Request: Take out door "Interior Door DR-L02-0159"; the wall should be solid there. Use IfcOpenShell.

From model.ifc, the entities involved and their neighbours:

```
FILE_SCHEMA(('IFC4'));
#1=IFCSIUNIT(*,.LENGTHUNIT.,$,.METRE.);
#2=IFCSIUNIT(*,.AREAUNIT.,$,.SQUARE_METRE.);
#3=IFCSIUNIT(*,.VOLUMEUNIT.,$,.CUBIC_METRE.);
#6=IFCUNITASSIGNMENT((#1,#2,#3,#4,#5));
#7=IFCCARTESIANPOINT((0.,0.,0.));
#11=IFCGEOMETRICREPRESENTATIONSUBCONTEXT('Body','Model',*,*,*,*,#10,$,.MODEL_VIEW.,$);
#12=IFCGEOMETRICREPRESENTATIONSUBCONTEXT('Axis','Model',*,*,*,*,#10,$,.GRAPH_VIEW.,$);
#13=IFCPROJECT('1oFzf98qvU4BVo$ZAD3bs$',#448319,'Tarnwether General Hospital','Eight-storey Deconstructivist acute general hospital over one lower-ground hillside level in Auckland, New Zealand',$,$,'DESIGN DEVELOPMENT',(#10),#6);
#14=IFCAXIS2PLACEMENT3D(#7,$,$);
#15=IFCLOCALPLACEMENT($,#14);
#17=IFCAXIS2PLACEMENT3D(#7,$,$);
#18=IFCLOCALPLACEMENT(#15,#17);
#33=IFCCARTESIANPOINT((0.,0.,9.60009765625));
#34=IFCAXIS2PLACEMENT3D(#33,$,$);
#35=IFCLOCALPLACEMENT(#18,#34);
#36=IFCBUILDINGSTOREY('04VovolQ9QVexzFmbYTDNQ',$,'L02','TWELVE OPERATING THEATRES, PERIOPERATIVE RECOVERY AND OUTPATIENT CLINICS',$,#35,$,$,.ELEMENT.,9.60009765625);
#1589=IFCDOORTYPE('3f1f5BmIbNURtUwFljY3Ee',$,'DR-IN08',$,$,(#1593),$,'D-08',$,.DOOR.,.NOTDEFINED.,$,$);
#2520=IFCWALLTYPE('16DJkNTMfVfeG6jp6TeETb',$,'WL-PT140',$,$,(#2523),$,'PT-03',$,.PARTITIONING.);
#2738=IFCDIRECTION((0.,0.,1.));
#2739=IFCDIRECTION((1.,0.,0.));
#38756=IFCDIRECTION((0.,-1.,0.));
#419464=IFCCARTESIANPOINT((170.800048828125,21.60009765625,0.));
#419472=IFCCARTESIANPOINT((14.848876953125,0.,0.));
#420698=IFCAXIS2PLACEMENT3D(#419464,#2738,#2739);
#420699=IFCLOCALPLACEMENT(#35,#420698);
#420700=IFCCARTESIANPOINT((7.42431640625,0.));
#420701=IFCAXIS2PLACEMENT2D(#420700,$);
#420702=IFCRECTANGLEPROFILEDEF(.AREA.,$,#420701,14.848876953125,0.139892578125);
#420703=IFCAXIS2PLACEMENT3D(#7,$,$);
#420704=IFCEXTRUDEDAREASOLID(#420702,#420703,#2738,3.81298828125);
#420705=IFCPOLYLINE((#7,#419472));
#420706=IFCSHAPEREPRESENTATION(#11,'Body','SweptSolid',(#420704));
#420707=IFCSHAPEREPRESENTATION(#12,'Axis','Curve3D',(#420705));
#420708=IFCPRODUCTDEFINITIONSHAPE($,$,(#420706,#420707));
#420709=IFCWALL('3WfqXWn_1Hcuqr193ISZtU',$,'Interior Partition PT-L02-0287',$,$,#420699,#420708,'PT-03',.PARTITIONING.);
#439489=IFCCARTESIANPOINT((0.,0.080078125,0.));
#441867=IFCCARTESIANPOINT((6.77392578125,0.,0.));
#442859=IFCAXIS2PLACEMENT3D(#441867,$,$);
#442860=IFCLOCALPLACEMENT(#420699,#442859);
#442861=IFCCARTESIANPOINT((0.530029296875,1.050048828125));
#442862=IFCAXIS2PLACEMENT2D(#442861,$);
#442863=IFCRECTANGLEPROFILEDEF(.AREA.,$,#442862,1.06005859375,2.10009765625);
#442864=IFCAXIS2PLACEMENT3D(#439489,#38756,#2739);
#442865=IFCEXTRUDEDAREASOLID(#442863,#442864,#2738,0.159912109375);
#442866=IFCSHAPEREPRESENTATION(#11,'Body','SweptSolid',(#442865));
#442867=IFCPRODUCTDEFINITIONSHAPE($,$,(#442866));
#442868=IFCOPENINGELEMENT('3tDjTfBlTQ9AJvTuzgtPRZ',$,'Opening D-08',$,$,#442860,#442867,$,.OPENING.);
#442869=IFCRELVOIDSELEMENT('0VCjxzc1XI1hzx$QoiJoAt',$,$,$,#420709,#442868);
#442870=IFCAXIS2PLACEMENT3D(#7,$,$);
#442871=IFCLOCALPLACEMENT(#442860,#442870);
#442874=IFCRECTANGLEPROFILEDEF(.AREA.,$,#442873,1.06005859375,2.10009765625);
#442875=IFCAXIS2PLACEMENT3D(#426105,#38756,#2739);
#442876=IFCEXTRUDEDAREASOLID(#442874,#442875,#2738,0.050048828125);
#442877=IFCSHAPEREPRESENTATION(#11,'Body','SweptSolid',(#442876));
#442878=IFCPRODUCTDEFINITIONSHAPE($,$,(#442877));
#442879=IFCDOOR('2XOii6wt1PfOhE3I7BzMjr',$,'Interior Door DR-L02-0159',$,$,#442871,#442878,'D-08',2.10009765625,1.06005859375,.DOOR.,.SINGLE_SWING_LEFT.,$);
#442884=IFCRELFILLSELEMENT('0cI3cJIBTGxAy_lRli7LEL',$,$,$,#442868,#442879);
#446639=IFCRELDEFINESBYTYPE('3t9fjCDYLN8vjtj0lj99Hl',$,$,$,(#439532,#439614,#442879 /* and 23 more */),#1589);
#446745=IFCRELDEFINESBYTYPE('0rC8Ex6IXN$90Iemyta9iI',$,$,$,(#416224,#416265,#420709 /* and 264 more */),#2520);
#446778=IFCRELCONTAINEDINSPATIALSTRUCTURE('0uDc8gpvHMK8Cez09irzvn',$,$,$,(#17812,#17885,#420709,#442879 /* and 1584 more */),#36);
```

```python
import ifcopenshell
import ifcopenshell.api.feature
import ifcopenshell.api.root
import ifcopenshell.geom
import ifcopenshell.util.shape

model = ifcopenshell.open("model.ifc")
settings = ifcopenshell.geom.settings()


def volume(element):
    """Net volume in cubic metres, openings subtracted."""
    shape = ifcopenshell.geom.create_shape(settings, element)
    return ifcopenshell.util.shape.get_volume(shape.geometry)


door = model.by_guid("2XOii6wt1PfOhE3I7BzMjr")
opening = door.FillsVoids[0].RelatingOpeningElement
wall = opening.VoidsElements[0].RelatingBuildingElement
before = volume(wall)

ifcopenshell.api.root.remove_product(model, product=door)
ifcopenshell.api.feature.remove_feature(model, feature=opening)

after = volume(wall)

print(f"wall volume {before:.3f} -> {after:.3f} m3")

model.write("model_rev.ifc")
```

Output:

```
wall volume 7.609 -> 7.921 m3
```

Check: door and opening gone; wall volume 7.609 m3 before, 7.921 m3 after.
